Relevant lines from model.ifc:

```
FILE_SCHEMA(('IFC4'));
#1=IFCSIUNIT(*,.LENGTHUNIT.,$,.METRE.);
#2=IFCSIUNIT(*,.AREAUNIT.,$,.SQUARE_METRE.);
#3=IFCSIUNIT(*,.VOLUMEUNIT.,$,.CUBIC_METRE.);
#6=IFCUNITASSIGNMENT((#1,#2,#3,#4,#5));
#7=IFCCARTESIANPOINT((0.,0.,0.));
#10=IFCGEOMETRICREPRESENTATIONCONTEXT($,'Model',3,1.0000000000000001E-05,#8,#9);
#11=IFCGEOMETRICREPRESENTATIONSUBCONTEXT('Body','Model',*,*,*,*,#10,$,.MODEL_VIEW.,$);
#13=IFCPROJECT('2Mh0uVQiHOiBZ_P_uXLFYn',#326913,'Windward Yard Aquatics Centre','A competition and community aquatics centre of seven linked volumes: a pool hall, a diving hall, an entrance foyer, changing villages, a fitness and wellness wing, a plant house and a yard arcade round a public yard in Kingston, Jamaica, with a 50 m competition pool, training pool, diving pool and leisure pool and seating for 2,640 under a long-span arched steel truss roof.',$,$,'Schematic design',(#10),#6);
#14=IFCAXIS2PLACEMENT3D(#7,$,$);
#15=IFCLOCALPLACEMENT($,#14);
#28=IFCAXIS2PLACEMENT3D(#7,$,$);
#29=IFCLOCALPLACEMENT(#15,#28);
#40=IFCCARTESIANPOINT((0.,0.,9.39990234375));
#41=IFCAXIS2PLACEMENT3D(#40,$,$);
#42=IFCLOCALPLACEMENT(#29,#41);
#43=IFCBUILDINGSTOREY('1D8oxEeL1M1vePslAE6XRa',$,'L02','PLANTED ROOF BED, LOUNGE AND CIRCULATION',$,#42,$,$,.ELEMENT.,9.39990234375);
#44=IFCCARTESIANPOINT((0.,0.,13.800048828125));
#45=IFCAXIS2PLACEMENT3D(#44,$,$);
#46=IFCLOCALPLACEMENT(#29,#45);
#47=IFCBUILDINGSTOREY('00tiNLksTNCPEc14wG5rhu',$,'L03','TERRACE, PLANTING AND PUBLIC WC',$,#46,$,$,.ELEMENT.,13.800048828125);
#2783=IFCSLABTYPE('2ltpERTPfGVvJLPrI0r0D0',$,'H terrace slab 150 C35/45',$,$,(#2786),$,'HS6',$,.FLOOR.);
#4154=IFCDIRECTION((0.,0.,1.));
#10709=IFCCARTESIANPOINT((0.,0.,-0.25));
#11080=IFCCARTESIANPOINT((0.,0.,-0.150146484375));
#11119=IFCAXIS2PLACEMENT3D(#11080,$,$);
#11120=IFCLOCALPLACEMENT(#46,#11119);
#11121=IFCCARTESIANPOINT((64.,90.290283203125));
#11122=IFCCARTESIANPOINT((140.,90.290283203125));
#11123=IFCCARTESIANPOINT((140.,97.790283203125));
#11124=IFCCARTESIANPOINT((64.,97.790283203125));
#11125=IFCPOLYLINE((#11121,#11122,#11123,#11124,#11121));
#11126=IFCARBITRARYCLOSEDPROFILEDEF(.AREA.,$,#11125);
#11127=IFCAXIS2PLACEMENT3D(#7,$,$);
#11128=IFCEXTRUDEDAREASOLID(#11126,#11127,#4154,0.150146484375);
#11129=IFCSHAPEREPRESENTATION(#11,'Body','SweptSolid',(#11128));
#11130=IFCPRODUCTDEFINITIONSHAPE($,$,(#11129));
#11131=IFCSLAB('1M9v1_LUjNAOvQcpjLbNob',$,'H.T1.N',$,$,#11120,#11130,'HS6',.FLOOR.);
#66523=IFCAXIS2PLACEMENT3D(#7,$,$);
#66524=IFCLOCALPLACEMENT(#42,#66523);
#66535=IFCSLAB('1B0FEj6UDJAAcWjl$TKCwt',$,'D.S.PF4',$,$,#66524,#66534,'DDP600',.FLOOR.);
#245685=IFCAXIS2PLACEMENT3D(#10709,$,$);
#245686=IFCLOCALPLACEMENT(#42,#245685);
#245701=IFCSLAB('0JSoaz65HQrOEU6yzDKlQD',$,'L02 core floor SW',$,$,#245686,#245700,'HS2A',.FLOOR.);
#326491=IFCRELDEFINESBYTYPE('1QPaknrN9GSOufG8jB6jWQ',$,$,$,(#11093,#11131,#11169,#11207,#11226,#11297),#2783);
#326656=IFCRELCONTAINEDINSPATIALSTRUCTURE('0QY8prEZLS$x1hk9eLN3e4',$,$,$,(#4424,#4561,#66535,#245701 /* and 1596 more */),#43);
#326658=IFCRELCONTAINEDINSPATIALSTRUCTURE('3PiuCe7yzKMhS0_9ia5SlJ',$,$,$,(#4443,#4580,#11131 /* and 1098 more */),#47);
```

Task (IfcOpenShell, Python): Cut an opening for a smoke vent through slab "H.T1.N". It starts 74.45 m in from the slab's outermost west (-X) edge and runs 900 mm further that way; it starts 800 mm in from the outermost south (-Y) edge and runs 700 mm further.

```python
import numpy as np
import ifcopenshell
import ifcopenshell.api.feature
import ifcopenshell.api.geometry
import ifcopenshell.api.root
import ifcopenshell.geom
import ifcopenshell.util.placement
import ifcopenshell.util.representation
import ifcopenshell.util.shape
import ifcopenshell.util.unit

model = ifcopenshell.open("model.ifc")
unit_scale = ifcopenshell.util.unit.calculate_unit_scale(model)
settings = ifcopenshell.geom.settings()


def volume(element):
    """Net volume in cubic metres, openings subtracted."""
    shape = ifcopenshell.geom.create_shape(settings, element)
    return ifcopenshell.util.shape.get_volume(shape.geometry)


slab = model.by_id(11131)
before = volume(slab)

# Extent in the slab's own axes, in metres. The edges named are its -X and -Y sides.
slab_shape = ifcopenshell.geom.create_shape(settings, slab)
vertices = ifcopenshell.util.shape.get_vertices(slab_shape.geometry)
x_min, y_min, bottom = vertices.min(axis=0)
top = vertices[:, 2].max()

opening = ifcopenshell.api.root.create_entity(model, ifc_class="IfcOpeningElement", name="Smoke vent opening", predefined_type="OPENING")
context = ifcopenshell.util.representation.get_context(model, "Model", "Body", "MODEL_VIEW")
width, depth = 0.9, 0.7
outline = [(0.0, 0.0), (width, 0.0), (width, depth), (0.0, depth), (0.0, 0.0)]
# Overshoot both faces by 50 mm so the cut is clean.
shape = ifcopenshell.api.geometry.add_slab_representation(
    model, context=context, depth=top - bottom + 0.1, polyline=outline
)
ifcopenshell.api.geometry.assign_representation(model, product=opening, representation=shape)

matrix = ifcopenshell.util.placement.get_local_placement(slab.ObjectPlacement)
matrix[:, 3] = matrix @ np.append(np.array([x_min + 74.45, y_min + 0.8, bottom - 0.05]) / unit_scale, 1.0)
ifcopenshell.api.geometry.edit_object_placement(model, product=opening, matrix=matrix, is_si=False)
ifcopenshell.api.feature.add_feature(model, feature=opening, element=slab)

after = volume(slab)

print(f"slab volume {before:.3f} -> {after:.3f} m3")

model.write("model-out.ifc")
```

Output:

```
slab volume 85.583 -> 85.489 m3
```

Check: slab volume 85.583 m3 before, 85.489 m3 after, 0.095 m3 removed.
